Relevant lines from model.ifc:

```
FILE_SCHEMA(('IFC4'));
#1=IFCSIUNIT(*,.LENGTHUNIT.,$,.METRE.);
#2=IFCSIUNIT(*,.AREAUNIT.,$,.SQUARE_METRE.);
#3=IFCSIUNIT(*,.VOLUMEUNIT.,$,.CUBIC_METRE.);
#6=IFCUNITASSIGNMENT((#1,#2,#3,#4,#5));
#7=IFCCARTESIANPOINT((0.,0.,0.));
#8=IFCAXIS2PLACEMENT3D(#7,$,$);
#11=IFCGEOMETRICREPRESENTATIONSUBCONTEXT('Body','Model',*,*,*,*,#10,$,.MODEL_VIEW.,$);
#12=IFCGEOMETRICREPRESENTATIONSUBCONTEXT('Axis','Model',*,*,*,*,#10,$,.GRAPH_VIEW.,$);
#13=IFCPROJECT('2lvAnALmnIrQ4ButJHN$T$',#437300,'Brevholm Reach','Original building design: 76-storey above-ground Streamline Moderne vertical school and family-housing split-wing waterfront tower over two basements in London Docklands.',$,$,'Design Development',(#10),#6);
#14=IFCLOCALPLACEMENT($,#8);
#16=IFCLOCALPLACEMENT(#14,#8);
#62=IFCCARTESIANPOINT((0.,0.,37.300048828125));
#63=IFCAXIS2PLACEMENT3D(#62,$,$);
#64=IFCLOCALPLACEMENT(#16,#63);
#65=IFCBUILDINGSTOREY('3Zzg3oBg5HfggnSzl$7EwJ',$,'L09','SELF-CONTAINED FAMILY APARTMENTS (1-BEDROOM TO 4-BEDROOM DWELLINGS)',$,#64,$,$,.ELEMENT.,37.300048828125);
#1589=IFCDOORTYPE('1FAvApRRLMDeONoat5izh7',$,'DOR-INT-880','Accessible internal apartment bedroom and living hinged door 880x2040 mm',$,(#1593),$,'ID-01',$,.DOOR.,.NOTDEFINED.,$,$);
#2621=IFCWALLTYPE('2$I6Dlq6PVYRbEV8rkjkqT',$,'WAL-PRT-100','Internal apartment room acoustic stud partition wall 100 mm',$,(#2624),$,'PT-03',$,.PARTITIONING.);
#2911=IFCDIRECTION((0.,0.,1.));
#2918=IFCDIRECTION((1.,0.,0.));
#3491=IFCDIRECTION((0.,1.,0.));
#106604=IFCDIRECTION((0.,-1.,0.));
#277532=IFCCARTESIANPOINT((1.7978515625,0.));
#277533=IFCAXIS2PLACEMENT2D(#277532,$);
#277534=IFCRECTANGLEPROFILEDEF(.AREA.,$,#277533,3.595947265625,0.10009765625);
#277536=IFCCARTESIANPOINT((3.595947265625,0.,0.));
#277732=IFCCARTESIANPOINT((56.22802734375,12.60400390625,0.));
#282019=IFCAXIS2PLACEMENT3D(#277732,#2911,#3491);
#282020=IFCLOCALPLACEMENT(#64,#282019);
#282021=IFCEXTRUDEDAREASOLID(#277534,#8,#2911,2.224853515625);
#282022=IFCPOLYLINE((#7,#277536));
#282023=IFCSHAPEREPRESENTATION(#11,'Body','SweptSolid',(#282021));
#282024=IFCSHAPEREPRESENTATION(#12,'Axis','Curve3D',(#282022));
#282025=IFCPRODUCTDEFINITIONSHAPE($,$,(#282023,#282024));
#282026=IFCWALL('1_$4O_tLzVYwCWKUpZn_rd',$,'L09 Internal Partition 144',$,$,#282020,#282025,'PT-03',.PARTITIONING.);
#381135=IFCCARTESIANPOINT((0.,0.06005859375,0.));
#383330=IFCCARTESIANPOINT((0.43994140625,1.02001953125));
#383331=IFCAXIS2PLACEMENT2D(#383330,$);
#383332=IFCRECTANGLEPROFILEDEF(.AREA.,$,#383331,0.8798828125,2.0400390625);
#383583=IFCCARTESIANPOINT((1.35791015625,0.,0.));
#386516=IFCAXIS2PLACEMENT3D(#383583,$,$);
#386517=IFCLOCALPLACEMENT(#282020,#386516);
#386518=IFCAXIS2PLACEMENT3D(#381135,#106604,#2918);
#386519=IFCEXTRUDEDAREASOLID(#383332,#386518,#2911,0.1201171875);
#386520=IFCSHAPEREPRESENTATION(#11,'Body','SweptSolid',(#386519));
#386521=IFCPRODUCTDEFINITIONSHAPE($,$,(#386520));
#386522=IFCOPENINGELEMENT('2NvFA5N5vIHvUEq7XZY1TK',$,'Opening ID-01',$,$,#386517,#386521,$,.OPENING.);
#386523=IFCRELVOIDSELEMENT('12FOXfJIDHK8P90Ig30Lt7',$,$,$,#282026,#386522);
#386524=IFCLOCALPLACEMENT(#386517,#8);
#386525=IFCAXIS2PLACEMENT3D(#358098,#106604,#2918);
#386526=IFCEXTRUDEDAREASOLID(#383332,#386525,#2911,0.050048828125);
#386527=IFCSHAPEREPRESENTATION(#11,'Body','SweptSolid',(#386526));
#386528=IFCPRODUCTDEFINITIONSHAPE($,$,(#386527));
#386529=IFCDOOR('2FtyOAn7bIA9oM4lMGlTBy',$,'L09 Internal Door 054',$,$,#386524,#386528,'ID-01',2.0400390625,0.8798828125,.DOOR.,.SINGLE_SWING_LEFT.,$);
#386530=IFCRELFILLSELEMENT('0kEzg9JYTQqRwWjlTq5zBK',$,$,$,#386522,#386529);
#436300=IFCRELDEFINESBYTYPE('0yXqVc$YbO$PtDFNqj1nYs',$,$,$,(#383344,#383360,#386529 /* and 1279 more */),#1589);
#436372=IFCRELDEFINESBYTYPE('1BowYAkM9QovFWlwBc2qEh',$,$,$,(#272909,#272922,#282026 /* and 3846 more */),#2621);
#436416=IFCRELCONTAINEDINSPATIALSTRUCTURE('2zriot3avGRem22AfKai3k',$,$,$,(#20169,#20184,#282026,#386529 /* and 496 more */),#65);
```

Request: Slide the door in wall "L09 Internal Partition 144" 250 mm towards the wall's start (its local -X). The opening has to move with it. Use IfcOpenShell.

```python
import ifcopenshell
import ifcopenshell.api.geometry
import ifcopenshell.util.placement

model = ifcopenshell.open("model.ifc")

door = model.by_id(386529)
opening = door.FillsVoids[0].RelatingOpeningElement
wall = opening.VoidsElements[0].RelatingBuildingElement

wall_matrix = ifcopenshell.util.placement.get_local_placement(wall.ObjectPlacement)
shift = wall_matrix[:3, 0] * -0.25
before = ifcopenshell.util.placement.get_local_placement(door.ObjectPlacement)[:3, 3].copy()

# The door is placed relative to its opening, so it follows when the opening moves.
matrix = ifcopenshell.util.placement.get_local_placement(opening.ObjectPlacement)
matrix[:3, 3] += shift
ifcopenshell.api.geometry.edit_object_placement(
    model, product=opening, matrix=matrix, is_si=False, should_transform_children=True
)

after = ifcopenshell.util.placement.get_local_placement(door.ObjectPlacement)[:3, 3]
print("door moved by", (after - before).round(3) + 0.0)

model.write("model_v2.ifc")
```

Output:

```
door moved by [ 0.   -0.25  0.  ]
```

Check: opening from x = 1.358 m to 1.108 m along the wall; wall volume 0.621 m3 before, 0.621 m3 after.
